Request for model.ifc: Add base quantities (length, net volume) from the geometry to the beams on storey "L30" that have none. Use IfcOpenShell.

First a look at what the model holds.

```python
import ifcopenshell
import ifcopenshell.util.element
import ifcopenshell.util.unit

model = ifcopenshell.open("model.ifc")
print(model.schema)
for unit_type in ("LENGTHUNIT", "AREAUNIT", "VOLUMEUNIT"):
    print(unit_type, ifcopenshell.util.unit.calculate_unit_scale(model, unit_type))
storey = next(s for s in model.by_type("IfcBuildingStorey") if s.Name == "L30")
beams = [e for e in ifcopenshell.util.element.get_decomposition(storey) if e.is_a("IfcBeam")]
for e in sorted(beams, key=lambda e: e.id()):
    print(e.id(), e.is_a(), e.Name, list(ifcopenshell.util.element.get_psets(e, qtos_only=True)), sep=" | ")
```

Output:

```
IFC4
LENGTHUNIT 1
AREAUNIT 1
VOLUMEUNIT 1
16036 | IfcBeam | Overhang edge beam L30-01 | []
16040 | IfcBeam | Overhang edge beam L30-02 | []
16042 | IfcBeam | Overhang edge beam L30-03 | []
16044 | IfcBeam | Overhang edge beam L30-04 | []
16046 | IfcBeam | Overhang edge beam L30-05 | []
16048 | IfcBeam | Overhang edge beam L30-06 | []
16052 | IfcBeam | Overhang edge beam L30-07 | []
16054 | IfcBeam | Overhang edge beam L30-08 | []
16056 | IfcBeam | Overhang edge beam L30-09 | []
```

```python
import ifcopenshell
import ifcopenshell.api.pset
import ifcopenshell.geom
import ifcopenshell.util.element
import ifcopenshell.util.shape
import ifcopenshell.util.unit

model = ifcopenshell.open("model.ifc")
unit_scale = ifcopenshell.util.unit.calculate_unit_scale(model)
volume_scale = ifcopenshell.util.unit.calculate_unit_scale(model, "VOLUMEUNIT")
settings = ifcopenshell.geom.settings()

storey = next(s for s in model.by_type("IfcBuildingStorey") if s.Name == "L30")
beams = [e for e in ifcopenshell.util.element.get_decomposition(storey) if e.is_a("IfcBeam")]

for e in sorted(beams, key=lambda e: e.id()):
    if ifcopenshell.util.element.get_psets(e, qtos_only=True, should_inherit=False):
        continue
    # Geometry comes back in metres, in the element's own axes.
    shape = ifcopenshell.geom.create_shape(settings, e)
    values = {
        "Length": ifcopenshell.util.shape.get_max_xyz(shape.geometry) / unit_scale,
        "NetVolume": ifcopenshell.util.shape.get_volume(shape.geometry) / volume_scale,
    }
    qto = ifcopenshell.api.pset.add_qto(model, product=e, name="Qto_BeamBaseQuantities")
    ifcopenshell.api.pset.edit_qto(model, qto=qto, properties=values)
    print(e.id(), {k: round(v, 3) for k, v in values.items()})

model.write("model_rev.ifc")
```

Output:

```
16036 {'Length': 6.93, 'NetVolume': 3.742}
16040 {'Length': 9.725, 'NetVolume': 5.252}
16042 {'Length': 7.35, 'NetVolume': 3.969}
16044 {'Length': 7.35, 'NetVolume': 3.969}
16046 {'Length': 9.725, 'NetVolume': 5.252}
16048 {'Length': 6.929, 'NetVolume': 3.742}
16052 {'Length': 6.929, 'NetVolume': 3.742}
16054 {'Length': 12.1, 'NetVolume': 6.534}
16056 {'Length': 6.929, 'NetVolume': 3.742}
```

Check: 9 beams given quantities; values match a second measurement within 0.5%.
